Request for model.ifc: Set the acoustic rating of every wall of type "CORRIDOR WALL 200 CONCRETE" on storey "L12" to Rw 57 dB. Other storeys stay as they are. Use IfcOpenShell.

First a look at what the model holds.

```python
import ifcopenshell
import ifcopenshell.util.element

model = ifcopenshell.open("model.ifc")
print(model.schema)
storey = next(s for s in model.by_type("IfcBuildingStorey") if s.Name == "L12")
walls = [e for e in ifcopenshell.util.element.get_decomposition(storey) if e.is_a("IfcWall")]
seen = {}
for e in walls:
    element_type = ifcopenshell.util.element.get_type(e)
    key = (element_type.Name if element_type != e and element_type else None, ifcopenshell.util.element.get_pset(e, "Pset_WallCommon", "AcousticRating"))
    seen[key] = seen.get(key, 0) + 1
for (name, value), count in sorted(seen.items(), key=str):
    print(count, "x", name, "|", value)
```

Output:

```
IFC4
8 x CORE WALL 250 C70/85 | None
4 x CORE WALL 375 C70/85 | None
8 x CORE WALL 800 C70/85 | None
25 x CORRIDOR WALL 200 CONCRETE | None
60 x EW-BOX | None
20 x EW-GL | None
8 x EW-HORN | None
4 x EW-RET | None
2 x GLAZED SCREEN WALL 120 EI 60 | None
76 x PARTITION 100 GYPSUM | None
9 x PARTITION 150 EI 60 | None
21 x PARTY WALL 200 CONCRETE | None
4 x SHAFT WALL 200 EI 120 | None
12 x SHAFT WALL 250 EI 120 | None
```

```python
import ifcopenshell
import ifcopenshell.api.pset
import ifcopenshell.util.element

model = ifcopenshell.open("model.ifc")

storey = next(s for s in model.by_type("IfcBuildingStorey") if s.Name == "L12")
walls = [e for e in ifcopenshell.util.element.get_decomposition(storey) if e.is_a("IfcWall")]

count = 0
for e in walls:
    element_type = ifcopenshell.util.element.get_type(e)
    if element_type in (None, e) or element_type.Name != "CORRIDOR WALL 200 CONCRETE":
        continue
    found = ifcopenshell.util.element.get_pset(e, "Pset_WallCommon", should_inherit=False)
    if found:
        pset = model.by_id(found["id"])
        if len(ifcopenshell.util.element.get_elements_by_pset(pset)) > 1:
            pset = ifcopenshell.api.pset.unshare_pset(model, products=[e], pset=pset)[0]
    else:
        pset = ifcopenshell.api.pset.add_pset(model, product=e, name="Pset_WallCommon")
    ifcopenshell.api.pset.edit_pset(model, pset=pset, properties={"AcousticRating": "Rw 57 dB"})
    count += 1

print(count, "walls updated")

model.write("model-out.ifc")
```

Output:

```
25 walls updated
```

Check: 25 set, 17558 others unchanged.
